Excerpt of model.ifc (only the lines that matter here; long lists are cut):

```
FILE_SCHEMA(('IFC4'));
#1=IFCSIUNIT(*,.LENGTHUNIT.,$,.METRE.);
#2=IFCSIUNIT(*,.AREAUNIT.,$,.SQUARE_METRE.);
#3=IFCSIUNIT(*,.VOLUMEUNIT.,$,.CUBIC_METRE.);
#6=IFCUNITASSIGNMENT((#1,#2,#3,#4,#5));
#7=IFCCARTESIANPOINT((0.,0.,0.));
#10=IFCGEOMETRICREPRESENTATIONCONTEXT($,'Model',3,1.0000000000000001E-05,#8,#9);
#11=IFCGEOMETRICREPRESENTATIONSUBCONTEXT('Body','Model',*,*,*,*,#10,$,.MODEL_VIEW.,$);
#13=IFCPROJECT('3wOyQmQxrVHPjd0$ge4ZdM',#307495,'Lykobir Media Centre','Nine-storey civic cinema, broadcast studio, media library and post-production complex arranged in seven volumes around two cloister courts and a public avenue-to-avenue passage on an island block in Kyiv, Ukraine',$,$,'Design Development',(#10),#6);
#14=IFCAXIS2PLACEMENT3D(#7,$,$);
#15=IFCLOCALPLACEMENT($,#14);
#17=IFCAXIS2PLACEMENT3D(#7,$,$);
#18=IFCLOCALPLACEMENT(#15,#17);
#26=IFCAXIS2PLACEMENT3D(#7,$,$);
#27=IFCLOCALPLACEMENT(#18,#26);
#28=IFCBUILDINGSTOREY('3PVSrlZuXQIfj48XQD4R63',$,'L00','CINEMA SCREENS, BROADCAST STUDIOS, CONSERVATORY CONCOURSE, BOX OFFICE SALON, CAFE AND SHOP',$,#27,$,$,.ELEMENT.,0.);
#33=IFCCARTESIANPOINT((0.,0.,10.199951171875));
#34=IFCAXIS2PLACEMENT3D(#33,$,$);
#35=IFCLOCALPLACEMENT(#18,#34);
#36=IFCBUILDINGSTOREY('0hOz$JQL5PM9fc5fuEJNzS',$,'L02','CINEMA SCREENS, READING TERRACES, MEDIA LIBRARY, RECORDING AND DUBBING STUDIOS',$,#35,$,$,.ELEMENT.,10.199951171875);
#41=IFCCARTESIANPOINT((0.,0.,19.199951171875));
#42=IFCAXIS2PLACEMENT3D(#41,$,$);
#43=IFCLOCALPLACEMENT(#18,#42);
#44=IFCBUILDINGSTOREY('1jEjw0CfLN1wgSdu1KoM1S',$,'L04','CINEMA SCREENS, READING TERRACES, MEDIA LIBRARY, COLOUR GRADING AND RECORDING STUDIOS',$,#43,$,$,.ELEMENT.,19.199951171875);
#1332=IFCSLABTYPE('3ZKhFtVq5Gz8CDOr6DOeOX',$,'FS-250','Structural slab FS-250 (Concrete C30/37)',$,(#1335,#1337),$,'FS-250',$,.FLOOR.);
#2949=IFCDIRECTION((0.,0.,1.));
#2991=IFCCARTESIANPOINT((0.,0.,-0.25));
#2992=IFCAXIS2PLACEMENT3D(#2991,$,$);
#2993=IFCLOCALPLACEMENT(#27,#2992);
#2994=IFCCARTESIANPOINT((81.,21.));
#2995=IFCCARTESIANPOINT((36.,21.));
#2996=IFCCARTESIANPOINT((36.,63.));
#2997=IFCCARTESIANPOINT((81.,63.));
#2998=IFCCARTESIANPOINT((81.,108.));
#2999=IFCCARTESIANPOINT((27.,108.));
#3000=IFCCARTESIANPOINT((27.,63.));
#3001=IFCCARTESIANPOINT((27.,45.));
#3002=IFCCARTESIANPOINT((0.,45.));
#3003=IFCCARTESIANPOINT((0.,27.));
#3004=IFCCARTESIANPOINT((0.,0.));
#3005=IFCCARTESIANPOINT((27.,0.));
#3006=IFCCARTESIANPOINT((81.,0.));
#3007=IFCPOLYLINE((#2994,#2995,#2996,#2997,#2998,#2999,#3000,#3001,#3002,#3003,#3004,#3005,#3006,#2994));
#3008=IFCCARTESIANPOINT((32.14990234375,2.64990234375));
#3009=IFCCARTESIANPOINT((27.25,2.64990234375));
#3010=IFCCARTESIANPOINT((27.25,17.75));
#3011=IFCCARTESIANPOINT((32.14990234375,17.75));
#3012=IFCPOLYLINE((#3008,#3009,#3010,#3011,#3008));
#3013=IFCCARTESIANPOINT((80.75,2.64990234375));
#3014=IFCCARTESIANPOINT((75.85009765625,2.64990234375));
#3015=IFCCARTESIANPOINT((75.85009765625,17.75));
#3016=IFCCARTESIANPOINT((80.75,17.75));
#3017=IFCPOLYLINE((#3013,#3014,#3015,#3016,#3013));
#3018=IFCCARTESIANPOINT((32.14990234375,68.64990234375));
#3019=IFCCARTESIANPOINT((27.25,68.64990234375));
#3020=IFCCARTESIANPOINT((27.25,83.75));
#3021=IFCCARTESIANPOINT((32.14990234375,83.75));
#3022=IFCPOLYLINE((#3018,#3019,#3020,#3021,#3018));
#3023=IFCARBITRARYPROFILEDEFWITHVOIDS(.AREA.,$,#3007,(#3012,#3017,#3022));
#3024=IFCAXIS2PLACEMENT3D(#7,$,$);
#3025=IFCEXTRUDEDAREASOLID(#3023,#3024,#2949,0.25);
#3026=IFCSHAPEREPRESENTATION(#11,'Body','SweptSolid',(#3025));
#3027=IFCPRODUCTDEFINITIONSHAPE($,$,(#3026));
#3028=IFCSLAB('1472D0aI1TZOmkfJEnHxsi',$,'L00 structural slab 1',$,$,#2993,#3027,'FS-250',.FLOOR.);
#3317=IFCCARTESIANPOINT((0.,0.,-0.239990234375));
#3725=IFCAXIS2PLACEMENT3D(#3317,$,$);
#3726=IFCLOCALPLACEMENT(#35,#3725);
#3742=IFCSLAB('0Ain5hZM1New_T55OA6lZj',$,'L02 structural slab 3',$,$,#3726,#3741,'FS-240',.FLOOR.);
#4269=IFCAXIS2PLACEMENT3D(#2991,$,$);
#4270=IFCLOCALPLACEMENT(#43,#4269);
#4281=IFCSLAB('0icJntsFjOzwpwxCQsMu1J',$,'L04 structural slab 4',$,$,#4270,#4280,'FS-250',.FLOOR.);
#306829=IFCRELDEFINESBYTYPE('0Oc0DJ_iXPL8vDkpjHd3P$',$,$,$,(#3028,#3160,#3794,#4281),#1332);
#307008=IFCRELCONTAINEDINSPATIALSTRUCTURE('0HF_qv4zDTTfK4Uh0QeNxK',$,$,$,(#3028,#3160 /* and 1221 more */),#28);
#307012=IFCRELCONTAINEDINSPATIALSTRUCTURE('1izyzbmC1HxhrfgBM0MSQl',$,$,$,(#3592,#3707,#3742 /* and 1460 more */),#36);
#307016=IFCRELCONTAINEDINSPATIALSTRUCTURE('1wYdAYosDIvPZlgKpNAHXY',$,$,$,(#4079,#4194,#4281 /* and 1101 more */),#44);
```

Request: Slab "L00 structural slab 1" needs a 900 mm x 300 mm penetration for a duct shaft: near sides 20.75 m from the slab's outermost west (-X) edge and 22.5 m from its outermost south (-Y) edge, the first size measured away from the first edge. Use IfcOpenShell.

```python
import numpy as np
import ifcopenshell
import ifcopenshell.api.feature
import ifcopenshell.api.geometry
import ifcopenshell.api.root
import ifcopenshell.geom
import ifcopenshell.util.placement
import ifcopenshell.util.representation
import ifcopenshell.util.shape
import ifcopenshell.util.unit

model = ifcopenshell.open("model.ifc")
unit_scale = ifcopenshell.util.unit.calculate_unit_scale(model)
settings = ifcopenshell.geom.settings()


def volume(element):
    """Net volume in cubic metres, openings subtracted."""
    shape = ifcopenshell.geom.create_shape(settings, element)
    return ifcopenshell.util.shape.get_volume(shape.geometry)


slab = model.by_guid("1472D0aI1TZOmkfJEnHxsi")
before = volume(slab)

# Extent in the slab's own axes, in metres. The edges named are its -X and -Y sides.
slab_shape = ifcopenshell.geom.create_shape(settings, slab)
vertices = ifcopenshell.util.shape.get_vertices(slab_shape.geometry)
x_min, y_min, bottom = vertices.min(axis=0)
top = vertices[:, 2].max()

opening = ifcopenshell.api.root.create_entity(model, ifc_class="IfcOpeningElement", name="Duct shaft opening", predefined_type="OPENING")
context = ifcopenshell.util.representation.get_context(model, "Model", "Body", "MODEL_VIEW")
width, depth = 0.9, 0.3
outline = [(0.0, 0.0), (width, 0.0), (width, depth), (0.0, depth), (0.0, 0.0)]
# Overshoot both faces by 50 mm so the cut is clean.
shape = ifcopenshell.api.geometry.add_slab_representation(
    model, context=context, depth=top - bottom + 0.1, polyline=outline
)
ifcopenshell.api.geometry.assign_representation(model, product=opening, representation=shape)

matrix = ifcopenshell.util.placement.get_local_placement(slab.ObjectPlacement)
matrix[:, 3] = matrix @ np.append(np.array([x_min + 20.75, y_min + 22.5, bottom - 0.05]) / unit_scale, 1.0)
ifcopenshell.api.geometry.edit_object_placement(model, product=opening, matrix=matrix, is_si=False)
ifcopenshell.api.feature.add_feature(model, feature=opening, element=slab)

after = volume(slab)

print(f"slab volume {before:.3f} -> {after:.3f} m3")

model.write("model_edited.ifc")
```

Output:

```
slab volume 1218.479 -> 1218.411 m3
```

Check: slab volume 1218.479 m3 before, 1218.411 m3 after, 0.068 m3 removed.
